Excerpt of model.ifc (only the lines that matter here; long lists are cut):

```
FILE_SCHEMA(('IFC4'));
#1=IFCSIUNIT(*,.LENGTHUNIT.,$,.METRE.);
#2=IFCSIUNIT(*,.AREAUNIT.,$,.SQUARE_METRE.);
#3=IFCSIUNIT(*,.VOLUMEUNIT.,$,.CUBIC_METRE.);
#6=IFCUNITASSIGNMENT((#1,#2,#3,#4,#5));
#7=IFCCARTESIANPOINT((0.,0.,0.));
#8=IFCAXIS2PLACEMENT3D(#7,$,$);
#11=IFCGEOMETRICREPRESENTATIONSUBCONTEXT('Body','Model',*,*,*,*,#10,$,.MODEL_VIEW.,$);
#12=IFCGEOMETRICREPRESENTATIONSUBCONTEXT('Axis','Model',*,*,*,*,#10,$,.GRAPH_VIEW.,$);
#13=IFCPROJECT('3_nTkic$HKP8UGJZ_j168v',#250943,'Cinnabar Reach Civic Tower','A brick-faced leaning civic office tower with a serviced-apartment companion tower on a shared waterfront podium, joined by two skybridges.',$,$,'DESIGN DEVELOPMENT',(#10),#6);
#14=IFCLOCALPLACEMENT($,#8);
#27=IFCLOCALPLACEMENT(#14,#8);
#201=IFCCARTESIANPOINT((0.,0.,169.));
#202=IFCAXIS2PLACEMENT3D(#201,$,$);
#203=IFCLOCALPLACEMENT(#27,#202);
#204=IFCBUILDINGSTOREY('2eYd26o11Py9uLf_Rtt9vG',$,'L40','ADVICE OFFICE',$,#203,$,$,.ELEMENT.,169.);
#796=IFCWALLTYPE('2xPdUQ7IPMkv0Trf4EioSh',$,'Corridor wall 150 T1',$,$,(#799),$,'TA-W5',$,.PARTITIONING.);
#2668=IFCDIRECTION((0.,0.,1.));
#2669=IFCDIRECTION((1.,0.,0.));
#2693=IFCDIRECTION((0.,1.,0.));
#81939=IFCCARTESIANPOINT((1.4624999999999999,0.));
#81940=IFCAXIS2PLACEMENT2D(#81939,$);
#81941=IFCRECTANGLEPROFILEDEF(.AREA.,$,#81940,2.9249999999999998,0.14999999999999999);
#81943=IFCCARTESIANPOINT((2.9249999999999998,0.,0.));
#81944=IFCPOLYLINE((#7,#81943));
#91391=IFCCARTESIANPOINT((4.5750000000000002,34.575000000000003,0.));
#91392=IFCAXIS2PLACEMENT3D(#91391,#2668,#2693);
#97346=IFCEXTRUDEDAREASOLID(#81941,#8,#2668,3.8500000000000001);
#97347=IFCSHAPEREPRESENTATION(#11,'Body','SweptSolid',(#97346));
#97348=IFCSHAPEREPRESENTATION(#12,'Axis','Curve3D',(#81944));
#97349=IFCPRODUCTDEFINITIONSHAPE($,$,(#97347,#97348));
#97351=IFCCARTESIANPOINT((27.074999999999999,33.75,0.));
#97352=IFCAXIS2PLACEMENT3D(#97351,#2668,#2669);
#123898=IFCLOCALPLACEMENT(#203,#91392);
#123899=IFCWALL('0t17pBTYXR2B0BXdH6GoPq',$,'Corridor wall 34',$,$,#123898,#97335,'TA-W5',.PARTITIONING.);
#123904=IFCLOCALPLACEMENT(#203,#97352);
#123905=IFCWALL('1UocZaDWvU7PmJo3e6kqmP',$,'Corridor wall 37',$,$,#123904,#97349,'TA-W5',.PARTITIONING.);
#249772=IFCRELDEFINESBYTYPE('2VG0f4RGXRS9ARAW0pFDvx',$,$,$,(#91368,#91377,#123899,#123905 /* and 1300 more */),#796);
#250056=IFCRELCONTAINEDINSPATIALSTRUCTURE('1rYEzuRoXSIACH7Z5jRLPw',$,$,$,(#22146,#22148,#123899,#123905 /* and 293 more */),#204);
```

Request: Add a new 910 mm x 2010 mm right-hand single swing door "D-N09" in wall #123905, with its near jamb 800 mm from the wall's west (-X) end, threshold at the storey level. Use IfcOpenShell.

```python
import numpy as np
import ifcopenshell
import ifcopenshell.api.feature
import ifcopenshell.api.geometry
import ifcopenshell.api.root
import ifcopenshell.api.spatial
import ifcopenshell.geom
import ifcopenshell.util.element
import ifcopenshell.util.placement
import ifcopenshell.util.representation
import ifcopenshell.util.shape
import ifcopenshell.util.unit

model = ifcopenshell.open("model.ifc")
unit_scale = ifcopenshell.util.unit.calculate_unit_scale(model)
settings = ifcopenshell.geom.settings()


def volume(element):
    """Net volume in cubic metres, openings subtracted."""
    shape = ifcopenshell.geom.create_shape(settings, element)
    return ifcopenshell.util.shape.get_volume(shape.geometry)


wall = model.by_id(123905)
storey = ifcopenshell.util.element.get_container(wall, ifc_class="IfcBuildingStorey")
context = ifcopenshell.util.representation.get_context(model, "Model", "Body", "MODEL_VIEW")
before = volume(wall)

width, height, from_end, sill = 0.91, 2.01, 0.8, 0.0  # metres

# The wall runs along its own X axis, and the end named is its -X end.
wall_shape = ifcopenshell.geom.create_shape(settings, wall)
x, y, z = ifcopenshell.util.shape.get_vertices(wall_shape.geometry).T
start = x.min() + from_end
face, thickness = float(y.min()), float(y.max() - y.min())
wall_matrix = ifcopenshell.util.placement.get_local_placement(wall.ObjectPlacement)
level = ifcopenshell.util.placement.get_local_placement(storey.ObjectPlacement)[2, 3]


def in_wall(x, y):
    """Placement at x, y metres in the wall's axes, at sill height."""
    matrix = wall_matrix.copy()
    matrix[:, 3] = wall_matrix @ np.array([x / unit_scale, y / unit_scale, 0.0, 1.0])
    matrix[2, 3] = level + sill / unit_scale
    return matrix


# Opening: a box that overshoots both wall faces by 50 mm.
opening = ifcopenshell.api.root.create_entity(model, ifc_class="IfcOpeningElement", predefined_type="OPENING")
box = ifcopenshell.api.geometry.add_wall_representation(
    model, context=context, length=width, height=height, thickness=thickness + 0.1
)
ifcopenshell.api.geometry.assign_representation(model, product=opening, representation=box)
ifcopenshell.api.geometry.edit_object_placement(model, product=opening, matrix=in_wall(start, face - 0.05), is_si=False)
ifcopenshell.api.feature.add_feature(model, feature=opening, element=wall)

door = ifcopenshell.api.root.create_entity(model, ifc_class="IfcDoor", name="D-N09", predefined_type="DOOR")
door.OverallWidth, door.OverallHeight = width / unit_scale, height / unit_scale
door.OperationType = "SINGLE_SWING_RIGHT"
body = ifcopenshell.api.geometry.add_door_representation(
    model,
    context=context,
    overall_width=door.OverallWidth,
    overall_height=door.OverallHeight,
    operation_type="SINGLE_SWING_RIGHT",
    lining_properties={"LiningDepth": thickness / unit_scale, "ThresholdDepth": thickness / unit_scale},
)
ifcopenshell.api.geometry.assign_representation(model, product=door, representation=body)
ifcopenshell.api.spatial.assign_container(model, products=[door], relating_structure=storey)
ifcopenshell.api.feature.add_filling(model, opening=opening, element=door)

# The lining spans the wall, so the door starts at the wall face.
ifcopenshell.api.geometry.edit_object_placement(model, product=door, matrix=in_wall(start, face), is_si=False)

after = volume(wall)

print(f"wall volume {before:.3f} -> {after:.3f} m3")

model.write("model_v2.ifc")
```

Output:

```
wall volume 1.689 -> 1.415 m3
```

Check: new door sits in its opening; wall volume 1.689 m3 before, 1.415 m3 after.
